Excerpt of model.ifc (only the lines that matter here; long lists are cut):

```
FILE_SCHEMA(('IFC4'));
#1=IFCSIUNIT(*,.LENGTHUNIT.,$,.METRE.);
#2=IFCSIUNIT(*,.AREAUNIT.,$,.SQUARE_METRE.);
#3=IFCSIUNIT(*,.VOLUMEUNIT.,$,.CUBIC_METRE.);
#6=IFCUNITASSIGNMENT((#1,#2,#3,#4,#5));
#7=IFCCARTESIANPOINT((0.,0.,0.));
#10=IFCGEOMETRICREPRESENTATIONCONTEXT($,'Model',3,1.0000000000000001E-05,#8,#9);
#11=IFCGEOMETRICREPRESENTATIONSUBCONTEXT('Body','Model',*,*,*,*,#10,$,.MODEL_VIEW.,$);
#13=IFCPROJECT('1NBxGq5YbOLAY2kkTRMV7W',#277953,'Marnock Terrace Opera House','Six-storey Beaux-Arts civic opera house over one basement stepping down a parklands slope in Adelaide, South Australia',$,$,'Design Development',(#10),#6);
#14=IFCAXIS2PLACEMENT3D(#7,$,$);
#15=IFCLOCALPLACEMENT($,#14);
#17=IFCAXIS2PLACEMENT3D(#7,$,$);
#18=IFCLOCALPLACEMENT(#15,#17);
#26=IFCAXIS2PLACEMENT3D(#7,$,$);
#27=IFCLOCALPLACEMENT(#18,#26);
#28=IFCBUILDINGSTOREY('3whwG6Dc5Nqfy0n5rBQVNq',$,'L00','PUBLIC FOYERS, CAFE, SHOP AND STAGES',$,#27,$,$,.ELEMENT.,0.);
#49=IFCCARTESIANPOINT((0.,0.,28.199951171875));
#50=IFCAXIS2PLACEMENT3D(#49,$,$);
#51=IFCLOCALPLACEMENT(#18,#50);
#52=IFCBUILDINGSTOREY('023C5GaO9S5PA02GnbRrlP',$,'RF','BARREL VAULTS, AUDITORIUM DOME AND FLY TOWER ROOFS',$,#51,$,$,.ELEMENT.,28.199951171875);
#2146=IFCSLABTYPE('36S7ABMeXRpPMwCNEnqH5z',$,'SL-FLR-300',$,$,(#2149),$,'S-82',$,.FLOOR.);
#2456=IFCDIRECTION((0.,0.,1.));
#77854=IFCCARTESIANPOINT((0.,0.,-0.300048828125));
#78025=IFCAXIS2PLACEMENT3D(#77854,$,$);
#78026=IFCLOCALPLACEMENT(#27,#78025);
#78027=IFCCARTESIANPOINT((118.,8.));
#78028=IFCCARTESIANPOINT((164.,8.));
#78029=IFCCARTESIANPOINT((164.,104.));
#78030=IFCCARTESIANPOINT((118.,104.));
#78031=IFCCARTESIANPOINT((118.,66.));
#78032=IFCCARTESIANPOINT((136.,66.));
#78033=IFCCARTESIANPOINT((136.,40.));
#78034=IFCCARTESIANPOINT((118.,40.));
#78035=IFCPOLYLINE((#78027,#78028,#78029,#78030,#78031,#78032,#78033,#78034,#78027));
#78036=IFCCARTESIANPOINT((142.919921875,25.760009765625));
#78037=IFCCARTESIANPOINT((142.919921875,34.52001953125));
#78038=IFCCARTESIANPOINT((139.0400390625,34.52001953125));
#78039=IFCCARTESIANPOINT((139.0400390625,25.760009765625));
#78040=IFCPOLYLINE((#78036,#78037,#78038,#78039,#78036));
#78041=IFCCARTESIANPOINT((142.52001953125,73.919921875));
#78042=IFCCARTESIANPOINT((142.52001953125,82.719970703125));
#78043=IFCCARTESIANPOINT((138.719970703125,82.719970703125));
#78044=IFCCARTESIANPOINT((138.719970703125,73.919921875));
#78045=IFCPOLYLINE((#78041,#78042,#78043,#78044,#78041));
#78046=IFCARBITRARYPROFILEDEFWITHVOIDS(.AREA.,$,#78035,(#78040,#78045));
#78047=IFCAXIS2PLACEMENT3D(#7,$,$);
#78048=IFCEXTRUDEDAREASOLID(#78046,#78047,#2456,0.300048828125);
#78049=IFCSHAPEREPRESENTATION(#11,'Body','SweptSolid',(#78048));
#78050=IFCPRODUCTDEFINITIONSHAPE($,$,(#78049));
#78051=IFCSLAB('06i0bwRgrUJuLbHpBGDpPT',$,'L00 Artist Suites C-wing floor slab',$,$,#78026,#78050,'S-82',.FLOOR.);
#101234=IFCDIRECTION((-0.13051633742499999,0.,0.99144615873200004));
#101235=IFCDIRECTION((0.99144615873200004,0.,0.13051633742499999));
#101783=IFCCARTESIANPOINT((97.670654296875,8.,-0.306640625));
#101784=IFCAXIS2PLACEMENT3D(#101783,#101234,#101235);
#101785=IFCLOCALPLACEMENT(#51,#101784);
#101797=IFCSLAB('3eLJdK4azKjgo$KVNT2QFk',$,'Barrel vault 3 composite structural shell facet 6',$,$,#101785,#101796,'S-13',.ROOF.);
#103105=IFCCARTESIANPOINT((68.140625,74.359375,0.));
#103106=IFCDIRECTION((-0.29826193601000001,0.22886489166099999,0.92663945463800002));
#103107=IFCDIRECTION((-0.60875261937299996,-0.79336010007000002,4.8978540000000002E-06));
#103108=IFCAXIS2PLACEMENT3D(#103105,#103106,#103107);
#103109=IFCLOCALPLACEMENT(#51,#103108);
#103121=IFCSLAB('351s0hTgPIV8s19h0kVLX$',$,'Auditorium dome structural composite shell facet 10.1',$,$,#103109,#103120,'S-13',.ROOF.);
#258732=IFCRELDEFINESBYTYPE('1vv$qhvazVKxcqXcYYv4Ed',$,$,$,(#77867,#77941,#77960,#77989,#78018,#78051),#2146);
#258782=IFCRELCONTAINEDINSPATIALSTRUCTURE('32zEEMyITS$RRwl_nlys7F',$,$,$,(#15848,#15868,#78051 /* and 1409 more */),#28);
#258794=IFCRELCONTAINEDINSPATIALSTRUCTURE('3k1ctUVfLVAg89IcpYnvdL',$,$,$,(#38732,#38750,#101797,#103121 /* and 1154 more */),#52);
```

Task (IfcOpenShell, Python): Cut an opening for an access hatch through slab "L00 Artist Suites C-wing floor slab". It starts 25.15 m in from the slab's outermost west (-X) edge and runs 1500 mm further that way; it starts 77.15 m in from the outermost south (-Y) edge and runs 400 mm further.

```python
import numpy as np
import ifcopenshell
import ifcopenshell.api.feature
import ifcopenshell.api.geometry
import ifcopenshell.api.root
import ifcopenshell.geom
import ifcopenshell.util.placement
import ifcopenshell.util.representation
import ifcopenshell.util.shape
import ifcopenshell.util.unit

model = ifcopenshell.open("model.ifc")
unit_scale = ifcopenshell.util.unit.calculate_unit_scale(model)
settings = ifcopenshell.geom.settings()


def volume(element):
    """Net volume in cubic metres, openings subtracted."""
    shape = ifcopenshell.geom.create_shape(settings, element)
    return ifcopenshell.util.shape.get_volume(shape.geometry)


slab = model.by_id(78051)
before = volume(slab)

# Extent in the slab's own axes, in metres. The edges named are its -X and -Y sides.
slab_shape = ifcopenshell.geom.create_shape(settings, slab)
vertices = ifcopenshell.util.shape.get_vertices(slab_shape.geometry)
x_min, y_min, bottom = vertices.min(axis=0)
top = vertices[:, 2].max()

opening = ifcopenshell.api.root.create_entity(model, ifc_class="IfcOpeningElement", name="Access hatch opening", predefined_type="OPENING")
context = ifcopenshell.util.representation.get_context(model, "Model", "Body", "MODEL_VIEW")
width, depth = 1.5, 0.4
outline = [(0.0, 0.0), (width, 0.0), (width, depth), (0.0, depth), (0.0, 0.0)]
# Overshoot both faces by 50 mm so the cut is clean.
shape = ifcopenshell.api.geometry.add_slab_representation(
    model, context=context, depth=top - bottom + 0.1, polyline=outline
)
ifcopenshell.api.geometry.assign_representation(model, product=opening, representation=shape)

matrix = ifcopenshell.util.placement.get_local_placement(slab.ObjectPlacement)
matrix[:, 3] = matrix @ np.append(np.array([x_min + 25.15, y_min + 77.15, bottom - 0.05]) / unit_scale, 1.0)
ifcopenshell.api.geometry.edit_object_placement(model, product=opening, matrix=matrix, is_si=False)
ifcopenshell.api.feature.add_feature(model, feature=opening, element=slab)

after = volume(slab)

print(f"slab volume {before:.3f} -> {after:.3f} m3")

model.write("model_rev.ifc")
```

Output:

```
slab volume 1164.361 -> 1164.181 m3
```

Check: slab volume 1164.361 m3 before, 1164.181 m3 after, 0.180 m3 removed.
